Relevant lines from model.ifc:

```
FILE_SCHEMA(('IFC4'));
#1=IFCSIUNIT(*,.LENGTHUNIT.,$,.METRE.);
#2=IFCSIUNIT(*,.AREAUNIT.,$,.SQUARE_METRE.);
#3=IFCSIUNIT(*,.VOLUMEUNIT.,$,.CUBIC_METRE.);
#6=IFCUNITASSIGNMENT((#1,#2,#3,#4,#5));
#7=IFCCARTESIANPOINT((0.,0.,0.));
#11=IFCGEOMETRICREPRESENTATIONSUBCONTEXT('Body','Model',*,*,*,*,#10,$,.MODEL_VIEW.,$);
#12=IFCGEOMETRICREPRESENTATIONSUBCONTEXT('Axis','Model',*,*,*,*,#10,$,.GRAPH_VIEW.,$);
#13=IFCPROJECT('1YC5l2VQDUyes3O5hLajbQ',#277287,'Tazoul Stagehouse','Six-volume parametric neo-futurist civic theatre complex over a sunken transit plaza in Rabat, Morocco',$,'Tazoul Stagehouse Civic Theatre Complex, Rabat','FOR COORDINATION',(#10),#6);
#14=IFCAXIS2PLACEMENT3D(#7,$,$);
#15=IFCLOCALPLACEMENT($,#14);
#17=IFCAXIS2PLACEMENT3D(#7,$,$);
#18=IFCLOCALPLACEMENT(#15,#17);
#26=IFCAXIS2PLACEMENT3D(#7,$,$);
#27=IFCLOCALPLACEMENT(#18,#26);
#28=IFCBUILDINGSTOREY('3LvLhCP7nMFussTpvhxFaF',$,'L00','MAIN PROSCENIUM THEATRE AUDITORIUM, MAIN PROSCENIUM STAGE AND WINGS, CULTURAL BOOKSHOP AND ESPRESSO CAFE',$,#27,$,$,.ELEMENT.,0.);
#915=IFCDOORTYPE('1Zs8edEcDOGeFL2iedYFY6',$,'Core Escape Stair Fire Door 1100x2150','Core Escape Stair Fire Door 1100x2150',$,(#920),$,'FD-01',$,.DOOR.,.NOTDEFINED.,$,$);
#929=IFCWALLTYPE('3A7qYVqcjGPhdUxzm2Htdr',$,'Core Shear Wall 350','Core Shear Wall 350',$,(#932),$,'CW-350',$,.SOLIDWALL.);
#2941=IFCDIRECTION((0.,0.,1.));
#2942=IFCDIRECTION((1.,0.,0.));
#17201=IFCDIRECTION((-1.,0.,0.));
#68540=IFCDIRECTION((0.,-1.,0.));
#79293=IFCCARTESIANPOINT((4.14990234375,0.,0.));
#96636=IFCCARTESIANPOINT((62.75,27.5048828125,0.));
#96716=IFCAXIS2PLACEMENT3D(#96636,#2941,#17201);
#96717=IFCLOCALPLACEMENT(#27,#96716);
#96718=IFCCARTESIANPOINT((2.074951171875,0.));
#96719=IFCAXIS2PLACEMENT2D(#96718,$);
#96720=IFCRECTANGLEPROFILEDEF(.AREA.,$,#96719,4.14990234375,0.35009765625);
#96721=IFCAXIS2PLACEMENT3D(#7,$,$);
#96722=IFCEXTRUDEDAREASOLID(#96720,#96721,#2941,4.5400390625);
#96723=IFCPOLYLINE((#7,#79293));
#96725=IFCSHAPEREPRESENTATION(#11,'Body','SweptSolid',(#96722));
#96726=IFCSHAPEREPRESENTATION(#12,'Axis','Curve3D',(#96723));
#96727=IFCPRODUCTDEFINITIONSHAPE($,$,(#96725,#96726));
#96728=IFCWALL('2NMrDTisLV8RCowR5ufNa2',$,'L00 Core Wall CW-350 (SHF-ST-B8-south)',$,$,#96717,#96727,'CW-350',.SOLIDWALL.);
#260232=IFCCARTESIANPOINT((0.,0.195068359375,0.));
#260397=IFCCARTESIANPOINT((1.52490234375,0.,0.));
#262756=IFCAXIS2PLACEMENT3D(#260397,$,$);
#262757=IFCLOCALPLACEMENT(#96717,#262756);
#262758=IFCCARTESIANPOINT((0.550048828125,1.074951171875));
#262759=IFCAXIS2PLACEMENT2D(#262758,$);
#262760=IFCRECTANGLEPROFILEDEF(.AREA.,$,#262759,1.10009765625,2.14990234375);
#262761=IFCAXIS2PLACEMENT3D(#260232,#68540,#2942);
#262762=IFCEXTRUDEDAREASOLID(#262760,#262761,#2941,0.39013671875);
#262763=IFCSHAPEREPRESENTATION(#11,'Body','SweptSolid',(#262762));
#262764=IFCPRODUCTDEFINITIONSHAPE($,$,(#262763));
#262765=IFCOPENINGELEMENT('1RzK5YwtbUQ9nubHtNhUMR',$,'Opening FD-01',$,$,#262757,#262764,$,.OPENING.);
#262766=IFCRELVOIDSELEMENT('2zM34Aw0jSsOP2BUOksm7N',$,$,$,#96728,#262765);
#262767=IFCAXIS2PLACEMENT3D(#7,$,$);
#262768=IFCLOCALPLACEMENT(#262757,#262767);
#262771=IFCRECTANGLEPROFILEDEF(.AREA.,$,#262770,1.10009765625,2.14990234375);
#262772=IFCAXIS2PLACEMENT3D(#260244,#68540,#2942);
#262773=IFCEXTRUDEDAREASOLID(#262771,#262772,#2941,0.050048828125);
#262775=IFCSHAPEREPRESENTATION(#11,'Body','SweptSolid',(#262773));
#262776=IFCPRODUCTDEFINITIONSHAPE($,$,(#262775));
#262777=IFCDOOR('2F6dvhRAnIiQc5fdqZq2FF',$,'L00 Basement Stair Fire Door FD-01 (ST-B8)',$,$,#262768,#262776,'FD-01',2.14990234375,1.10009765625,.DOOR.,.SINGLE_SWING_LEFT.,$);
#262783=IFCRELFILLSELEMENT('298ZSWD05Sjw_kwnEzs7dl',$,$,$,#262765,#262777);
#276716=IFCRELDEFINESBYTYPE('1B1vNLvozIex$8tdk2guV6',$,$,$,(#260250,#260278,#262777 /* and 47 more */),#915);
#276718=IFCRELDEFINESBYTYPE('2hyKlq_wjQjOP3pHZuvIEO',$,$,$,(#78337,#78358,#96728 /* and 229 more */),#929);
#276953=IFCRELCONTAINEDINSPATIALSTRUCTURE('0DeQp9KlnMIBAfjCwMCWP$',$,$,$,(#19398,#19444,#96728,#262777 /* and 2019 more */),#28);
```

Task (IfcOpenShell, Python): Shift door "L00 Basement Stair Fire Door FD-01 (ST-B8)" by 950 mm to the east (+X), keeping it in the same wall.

```python
import ifcopenshell
import ifcopenshell.api.geometry
import ifcopenshell.util.placement

model = ifcopenshell.open("model.ifc")

door = model.by_guid("2F6dvhRAnIiQc5fdqZq2FF")
opening = door.FillsVoids[0].RelatingOpeningElement
wall = opening.VoidsElements[0].RelatingBuildingElement

wall_matrix = ifcopenshell.util.placement.get_local_placement(wall.ObjectPlacement)
shift = wall_matrix[:3, 0] * -0.95
before = ifcopenshell.util.placement.get_local_placement(door.ObjectPlacement)[:3, 3].copy()

# The door is placed relative to its opening, so it follows when the opening moves.
matrix = ifcopenshell.util.placement.get_local_placement(opening.ObjectPlacement)
matrix[:3, 3] += shift
ifcopenshell.api.geometry.edit_object_placement(
    model, product=opening, matrix=matrix, is_si=False, should_transform_children=True
)

after = ifcopenshell.util.placement.get_local_placement(door.ObjectPlacement)[:3, 3]
print("door moved by", (after - before).round(3) + 0.0)

model.write("model_v2.ifc")
```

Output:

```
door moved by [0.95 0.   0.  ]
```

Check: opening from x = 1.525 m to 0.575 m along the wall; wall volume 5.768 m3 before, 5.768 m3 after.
